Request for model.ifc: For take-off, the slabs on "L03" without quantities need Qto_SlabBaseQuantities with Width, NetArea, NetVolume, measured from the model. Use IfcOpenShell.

First a look at what the model holds.

```python
import ifcopenshell
import ifcopenshell.util.element
import ifcopenshell.util.unit

model = ifcopenshell.open("model.ifc")
print(model.schema)
for unit_type in ("LENGTHUNIT", "AREAUNIT", "VOLUMEUNIT"):
    print(unit_type, ifcopenshell.util.unit.calculate_unit_scale(model, unit_type))
storey = next(s for s in model.by_type("IfcBuildingStorey") if s.Name == "L03")
slabs = [e for e in ifcopenshell.util.element.get_decomposition(storey) if e.is_a("IfcSlab")]
for e in sorted(slabs, key=lambda e: e.id()):
    print(e.id(), e.is_a(), e.Name, list(ifcopenshell.util.element.get_psets(e, qtos_only=True)), sep=" | ")
```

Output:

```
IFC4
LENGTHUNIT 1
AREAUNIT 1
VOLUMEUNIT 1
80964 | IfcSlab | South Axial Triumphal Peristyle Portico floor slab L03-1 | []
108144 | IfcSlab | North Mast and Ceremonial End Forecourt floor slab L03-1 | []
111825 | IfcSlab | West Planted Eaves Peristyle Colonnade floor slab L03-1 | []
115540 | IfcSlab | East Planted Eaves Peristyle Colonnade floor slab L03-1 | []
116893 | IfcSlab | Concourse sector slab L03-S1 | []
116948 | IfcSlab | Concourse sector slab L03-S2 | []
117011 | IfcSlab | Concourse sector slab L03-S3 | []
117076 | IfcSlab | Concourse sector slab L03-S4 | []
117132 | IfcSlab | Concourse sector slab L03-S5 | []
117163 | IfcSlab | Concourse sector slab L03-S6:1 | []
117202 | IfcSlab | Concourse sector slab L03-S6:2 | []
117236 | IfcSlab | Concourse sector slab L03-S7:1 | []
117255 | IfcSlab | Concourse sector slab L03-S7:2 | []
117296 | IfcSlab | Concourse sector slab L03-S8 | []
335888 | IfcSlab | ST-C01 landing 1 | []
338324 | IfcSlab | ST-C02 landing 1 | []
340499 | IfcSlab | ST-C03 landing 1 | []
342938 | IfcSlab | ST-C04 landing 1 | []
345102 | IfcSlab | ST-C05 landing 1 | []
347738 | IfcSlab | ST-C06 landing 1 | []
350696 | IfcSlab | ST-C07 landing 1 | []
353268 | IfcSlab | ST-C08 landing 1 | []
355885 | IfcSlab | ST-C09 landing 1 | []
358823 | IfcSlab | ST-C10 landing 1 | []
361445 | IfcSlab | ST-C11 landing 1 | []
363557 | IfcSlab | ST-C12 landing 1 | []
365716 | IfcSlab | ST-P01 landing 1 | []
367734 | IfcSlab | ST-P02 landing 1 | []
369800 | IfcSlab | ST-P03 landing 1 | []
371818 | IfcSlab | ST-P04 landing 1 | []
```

```python
import ifcopenshell
import ifcopenshell.api.pset
import ifcopenshell.geom
import ifcopenshell.util.element
import ifcopenshell.util.shape
import ifcopenshell.util.unit

model = ifcopenshell.open("model.ifc")
unit_scale = ifcopenshell.util.unit.calculate_unit_scale(model)
area_scale = ifcopenshell.util.unit.calculate_unit_scale(model, "AREAUNIT")
volume_scale = ifcopenshell.util.unit.calculate_unit_scale(model, "VOLUMEUNIT")
settings = ifcopenshell.geom.settings()

storey = next(s for s in model.by_type("IfcBuildingStorey") if s.Name == "L03")
slabs = [e for e in ifcopenshell.util.element.get_decomposition(storey) if e.is_a("IfcSlab")]

for e in sorted(slabs, key=lambda e: e.id()):
    if ifcopenshell.util.element.get_psets(e, qtos_only=True, should_inherit=False):
        continue
    # Geometry comes back in metres, in the element's own axes.
    shape = ifcopenshell.geom.create_shape(settings, e)
    values = {
        "Width": ifcopenshell.util.shape.get_z(shape.geometry) / unit_scale,
        "NetArea": ifcopenshell.util.shape.get_footprint_area(shape.geometry) / area_scale,
        "NetVolume": ifcopenshell.util.shape.get_volume(shape.geometry) / volume_scale,
    }
    qto = ifcopenshell.api.pset.add_qto(model, product=e, name="Qto_SlabBaseQuantities")
    ifcopenshell.api.pset.edit_qto(model, qto=qto, properties=values)
    print(e.id(), {k: round(v, 3) for k, v in values.items()})

model.write("model_updated.ifc")
```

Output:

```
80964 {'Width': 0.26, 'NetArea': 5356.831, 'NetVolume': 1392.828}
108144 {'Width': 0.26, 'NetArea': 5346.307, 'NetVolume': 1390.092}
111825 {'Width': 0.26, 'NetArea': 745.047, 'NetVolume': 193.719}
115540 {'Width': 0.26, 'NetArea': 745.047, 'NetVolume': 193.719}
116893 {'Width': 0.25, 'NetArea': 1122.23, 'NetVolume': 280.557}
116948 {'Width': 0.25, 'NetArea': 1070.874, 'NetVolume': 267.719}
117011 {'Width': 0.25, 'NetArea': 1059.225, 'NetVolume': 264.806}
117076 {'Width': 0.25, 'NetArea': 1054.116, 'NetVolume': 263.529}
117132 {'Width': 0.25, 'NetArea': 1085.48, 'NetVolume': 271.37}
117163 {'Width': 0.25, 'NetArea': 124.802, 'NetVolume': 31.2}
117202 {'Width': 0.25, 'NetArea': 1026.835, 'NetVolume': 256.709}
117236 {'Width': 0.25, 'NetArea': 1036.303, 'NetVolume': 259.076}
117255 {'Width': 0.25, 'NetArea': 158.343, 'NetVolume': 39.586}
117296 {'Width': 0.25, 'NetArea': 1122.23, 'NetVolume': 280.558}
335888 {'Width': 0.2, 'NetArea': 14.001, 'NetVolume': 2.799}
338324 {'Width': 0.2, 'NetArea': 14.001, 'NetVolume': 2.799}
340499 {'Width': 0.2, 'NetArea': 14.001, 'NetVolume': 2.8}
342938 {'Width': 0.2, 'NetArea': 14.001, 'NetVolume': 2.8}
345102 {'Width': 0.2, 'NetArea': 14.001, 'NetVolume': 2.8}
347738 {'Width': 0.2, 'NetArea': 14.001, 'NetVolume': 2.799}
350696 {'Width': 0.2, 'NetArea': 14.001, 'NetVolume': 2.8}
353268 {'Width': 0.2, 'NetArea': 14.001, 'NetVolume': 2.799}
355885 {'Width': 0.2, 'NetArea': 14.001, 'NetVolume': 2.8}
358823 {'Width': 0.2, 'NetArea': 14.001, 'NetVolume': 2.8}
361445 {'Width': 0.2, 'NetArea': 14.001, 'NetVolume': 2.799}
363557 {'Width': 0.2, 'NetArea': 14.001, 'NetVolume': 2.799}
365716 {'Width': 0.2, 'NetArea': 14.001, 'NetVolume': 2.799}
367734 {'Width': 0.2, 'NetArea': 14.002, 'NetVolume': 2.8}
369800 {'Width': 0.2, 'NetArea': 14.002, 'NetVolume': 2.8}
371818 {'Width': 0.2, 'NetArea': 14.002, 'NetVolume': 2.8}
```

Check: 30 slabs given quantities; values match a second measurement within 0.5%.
